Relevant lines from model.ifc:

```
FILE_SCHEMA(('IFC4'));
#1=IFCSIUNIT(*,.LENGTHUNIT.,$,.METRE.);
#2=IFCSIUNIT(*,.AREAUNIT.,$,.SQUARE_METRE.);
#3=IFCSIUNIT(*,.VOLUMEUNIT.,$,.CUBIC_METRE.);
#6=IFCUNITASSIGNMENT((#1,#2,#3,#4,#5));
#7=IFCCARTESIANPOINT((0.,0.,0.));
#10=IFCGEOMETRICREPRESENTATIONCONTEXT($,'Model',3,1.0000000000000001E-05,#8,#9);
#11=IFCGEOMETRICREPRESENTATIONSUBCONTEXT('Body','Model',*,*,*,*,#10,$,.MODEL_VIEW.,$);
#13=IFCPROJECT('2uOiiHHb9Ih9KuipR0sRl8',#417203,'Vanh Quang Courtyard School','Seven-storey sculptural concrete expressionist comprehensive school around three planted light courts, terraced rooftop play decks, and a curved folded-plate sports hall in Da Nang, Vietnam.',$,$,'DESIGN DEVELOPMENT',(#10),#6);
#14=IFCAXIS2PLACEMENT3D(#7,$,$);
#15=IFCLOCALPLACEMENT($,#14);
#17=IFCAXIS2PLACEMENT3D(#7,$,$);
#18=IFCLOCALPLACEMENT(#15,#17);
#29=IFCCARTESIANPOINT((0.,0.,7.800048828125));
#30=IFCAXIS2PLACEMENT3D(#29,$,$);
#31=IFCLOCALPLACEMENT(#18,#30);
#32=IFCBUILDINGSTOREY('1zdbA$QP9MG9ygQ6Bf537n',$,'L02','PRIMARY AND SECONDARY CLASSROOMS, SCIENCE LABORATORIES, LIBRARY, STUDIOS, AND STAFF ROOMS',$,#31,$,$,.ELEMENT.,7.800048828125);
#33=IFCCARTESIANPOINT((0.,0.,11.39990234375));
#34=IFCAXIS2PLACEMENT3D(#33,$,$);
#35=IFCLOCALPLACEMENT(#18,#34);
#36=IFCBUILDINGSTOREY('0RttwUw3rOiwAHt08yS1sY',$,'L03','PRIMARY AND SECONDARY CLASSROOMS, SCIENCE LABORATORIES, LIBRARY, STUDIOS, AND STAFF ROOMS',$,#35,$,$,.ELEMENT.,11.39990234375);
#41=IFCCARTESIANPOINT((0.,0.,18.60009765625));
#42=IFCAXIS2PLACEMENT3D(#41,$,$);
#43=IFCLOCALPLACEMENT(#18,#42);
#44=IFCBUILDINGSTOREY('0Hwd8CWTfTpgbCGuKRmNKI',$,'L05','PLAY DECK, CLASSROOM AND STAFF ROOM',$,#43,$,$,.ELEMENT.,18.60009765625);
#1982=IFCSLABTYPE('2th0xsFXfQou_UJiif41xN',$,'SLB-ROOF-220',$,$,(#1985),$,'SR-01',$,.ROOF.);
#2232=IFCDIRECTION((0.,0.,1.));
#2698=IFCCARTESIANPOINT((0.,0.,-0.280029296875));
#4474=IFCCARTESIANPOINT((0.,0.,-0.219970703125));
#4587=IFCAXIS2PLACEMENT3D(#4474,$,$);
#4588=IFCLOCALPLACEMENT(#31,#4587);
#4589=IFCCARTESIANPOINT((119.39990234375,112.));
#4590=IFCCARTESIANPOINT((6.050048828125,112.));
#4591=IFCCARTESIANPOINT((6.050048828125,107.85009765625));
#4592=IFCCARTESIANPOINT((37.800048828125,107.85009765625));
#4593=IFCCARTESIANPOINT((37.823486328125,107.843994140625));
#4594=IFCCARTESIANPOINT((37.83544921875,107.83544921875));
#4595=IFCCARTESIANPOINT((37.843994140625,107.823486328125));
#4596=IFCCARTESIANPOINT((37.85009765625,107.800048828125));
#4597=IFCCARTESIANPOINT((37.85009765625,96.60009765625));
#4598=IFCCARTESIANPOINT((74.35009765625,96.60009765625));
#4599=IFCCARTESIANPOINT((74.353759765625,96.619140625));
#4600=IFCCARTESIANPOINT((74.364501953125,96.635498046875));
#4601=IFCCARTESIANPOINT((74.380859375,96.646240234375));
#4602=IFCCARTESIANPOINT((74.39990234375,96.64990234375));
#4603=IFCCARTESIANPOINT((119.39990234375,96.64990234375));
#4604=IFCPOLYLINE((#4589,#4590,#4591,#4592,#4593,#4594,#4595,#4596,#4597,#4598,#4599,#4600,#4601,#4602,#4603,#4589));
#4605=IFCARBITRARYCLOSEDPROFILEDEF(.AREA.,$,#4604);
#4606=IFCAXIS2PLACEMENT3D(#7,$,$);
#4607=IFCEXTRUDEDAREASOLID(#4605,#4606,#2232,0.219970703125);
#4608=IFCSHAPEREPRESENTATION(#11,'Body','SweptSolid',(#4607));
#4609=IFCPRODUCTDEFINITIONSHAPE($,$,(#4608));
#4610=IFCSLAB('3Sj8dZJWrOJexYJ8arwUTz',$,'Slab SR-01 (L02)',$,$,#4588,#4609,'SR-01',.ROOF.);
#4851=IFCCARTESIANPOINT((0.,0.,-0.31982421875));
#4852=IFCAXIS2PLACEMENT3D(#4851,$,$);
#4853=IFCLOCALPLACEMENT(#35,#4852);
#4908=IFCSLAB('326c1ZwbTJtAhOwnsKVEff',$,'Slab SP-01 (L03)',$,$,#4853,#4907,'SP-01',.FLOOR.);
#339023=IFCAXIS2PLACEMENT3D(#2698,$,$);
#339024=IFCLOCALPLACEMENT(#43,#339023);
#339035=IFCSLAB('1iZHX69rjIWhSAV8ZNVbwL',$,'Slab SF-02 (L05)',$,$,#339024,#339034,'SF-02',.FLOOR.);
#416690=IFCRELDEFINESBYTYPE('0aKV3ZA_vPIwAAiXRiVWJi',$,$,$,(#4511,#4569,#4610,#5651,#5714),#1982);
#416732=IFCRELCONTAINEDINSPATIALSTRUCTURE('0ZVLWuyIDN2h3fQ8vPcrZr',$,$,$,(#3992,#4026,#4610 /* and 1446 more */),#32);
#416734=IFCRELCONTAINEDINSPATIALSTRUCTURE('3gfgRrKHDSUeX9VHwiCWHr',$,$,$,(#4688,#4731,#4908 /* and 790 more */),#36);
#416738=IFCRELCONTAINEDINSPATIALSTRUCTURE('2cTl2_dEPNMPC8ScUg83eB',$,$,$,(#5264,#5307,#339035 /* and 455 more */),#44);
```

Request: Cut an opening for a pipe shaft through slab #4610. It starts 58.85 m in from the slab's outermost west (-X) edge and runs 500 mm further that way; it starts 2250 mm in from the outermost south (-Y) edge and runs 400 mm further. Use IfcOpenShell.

```python
import numpy as np
import ifcopenshell
import ifcopenshell.api.feature
import ifcopenshell.api.geometry
import ifcopenshell.api.root
import ifcopenshell.geom
import ifcopenshell.util.placement
import ifcopenshell.util.representation
import ifcopenshell.util.shape
import ifcopenshell.util.unit

model = ifcopenshell.open("model.ifc")
unit_scale = ifcopenshell.util.unit.calculate_unit_scale(model)
settings = ifcopenshell.geom.settings()


def volume(element):
    """Net volume in cubic metres, openings subtracted."""
    shape = ifcopenshell.geom.create_shape(settings, element)
    return ifcopenshell.util.shape.get_volume(shape.geometry)


slab = model.by_guid("3Sj8dZJWrOJexYJ8arwUTz")
before = volume(slab)

# Extent in the slab's own axes, in metres. The edges named are its -X and -Y sides.
slab_shape = ifcopenshell.geom.create_shape(settings, slab)
vertices = ifcopenshell.util.shape.get_vertices(slab_shape.geometry)
x_min, y_min, bottom = vertices.min(axis=0)
top = vertices[:, 2].max()

opening = ifcopenshell.api.root.create_entity(model, ifc_class="IfcOpeningElement", name="Pipe shaft opening", predefined_type="OPENING")
context = ifcopenshell.util.representation.get_context(model, "Model", "Body", "MODEL_VIEW")
width, depth = 0.5, 0.4
outline = [(0.0, 0.0), (width, 0.0), (width, depth), (0.0, depth), (0.0, 0.0)]
# Overshoot both faces by 50 mm so the cut is clean.
shape = ifcopenshell.api.geometry.add_slab_representation(
    model, context=context, depth=top - bottom + 0.1, polyline=outline
)
ifcopenshell.api.geometry.assign_representation(model, product=opening, representation=shape)

matrix = ifcopenshell.util.placement.get_local_placement(slab.ObjectPlacement)
matrix[:, 3] = matrix @ np.append(np.array([x_min + 58.85, y_min + 2.25, bottom - 0.05]) / unit_scale, 1.0)
ifcopenshell.api.geometry.edit_object_placement(model, product=opening, matrix=matrix, is_si=False)
ifcopenshell.api.feature.add_feature(model, feature=opening, element=slab)

after = volume(slab)

print(f"slab volume {before:.3f} -> {after:.3f} m3")

model.write("model_edited.ifc")
```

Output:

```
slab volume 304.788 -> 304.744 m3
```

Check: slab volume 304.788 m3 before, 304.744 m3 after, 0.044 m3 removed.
